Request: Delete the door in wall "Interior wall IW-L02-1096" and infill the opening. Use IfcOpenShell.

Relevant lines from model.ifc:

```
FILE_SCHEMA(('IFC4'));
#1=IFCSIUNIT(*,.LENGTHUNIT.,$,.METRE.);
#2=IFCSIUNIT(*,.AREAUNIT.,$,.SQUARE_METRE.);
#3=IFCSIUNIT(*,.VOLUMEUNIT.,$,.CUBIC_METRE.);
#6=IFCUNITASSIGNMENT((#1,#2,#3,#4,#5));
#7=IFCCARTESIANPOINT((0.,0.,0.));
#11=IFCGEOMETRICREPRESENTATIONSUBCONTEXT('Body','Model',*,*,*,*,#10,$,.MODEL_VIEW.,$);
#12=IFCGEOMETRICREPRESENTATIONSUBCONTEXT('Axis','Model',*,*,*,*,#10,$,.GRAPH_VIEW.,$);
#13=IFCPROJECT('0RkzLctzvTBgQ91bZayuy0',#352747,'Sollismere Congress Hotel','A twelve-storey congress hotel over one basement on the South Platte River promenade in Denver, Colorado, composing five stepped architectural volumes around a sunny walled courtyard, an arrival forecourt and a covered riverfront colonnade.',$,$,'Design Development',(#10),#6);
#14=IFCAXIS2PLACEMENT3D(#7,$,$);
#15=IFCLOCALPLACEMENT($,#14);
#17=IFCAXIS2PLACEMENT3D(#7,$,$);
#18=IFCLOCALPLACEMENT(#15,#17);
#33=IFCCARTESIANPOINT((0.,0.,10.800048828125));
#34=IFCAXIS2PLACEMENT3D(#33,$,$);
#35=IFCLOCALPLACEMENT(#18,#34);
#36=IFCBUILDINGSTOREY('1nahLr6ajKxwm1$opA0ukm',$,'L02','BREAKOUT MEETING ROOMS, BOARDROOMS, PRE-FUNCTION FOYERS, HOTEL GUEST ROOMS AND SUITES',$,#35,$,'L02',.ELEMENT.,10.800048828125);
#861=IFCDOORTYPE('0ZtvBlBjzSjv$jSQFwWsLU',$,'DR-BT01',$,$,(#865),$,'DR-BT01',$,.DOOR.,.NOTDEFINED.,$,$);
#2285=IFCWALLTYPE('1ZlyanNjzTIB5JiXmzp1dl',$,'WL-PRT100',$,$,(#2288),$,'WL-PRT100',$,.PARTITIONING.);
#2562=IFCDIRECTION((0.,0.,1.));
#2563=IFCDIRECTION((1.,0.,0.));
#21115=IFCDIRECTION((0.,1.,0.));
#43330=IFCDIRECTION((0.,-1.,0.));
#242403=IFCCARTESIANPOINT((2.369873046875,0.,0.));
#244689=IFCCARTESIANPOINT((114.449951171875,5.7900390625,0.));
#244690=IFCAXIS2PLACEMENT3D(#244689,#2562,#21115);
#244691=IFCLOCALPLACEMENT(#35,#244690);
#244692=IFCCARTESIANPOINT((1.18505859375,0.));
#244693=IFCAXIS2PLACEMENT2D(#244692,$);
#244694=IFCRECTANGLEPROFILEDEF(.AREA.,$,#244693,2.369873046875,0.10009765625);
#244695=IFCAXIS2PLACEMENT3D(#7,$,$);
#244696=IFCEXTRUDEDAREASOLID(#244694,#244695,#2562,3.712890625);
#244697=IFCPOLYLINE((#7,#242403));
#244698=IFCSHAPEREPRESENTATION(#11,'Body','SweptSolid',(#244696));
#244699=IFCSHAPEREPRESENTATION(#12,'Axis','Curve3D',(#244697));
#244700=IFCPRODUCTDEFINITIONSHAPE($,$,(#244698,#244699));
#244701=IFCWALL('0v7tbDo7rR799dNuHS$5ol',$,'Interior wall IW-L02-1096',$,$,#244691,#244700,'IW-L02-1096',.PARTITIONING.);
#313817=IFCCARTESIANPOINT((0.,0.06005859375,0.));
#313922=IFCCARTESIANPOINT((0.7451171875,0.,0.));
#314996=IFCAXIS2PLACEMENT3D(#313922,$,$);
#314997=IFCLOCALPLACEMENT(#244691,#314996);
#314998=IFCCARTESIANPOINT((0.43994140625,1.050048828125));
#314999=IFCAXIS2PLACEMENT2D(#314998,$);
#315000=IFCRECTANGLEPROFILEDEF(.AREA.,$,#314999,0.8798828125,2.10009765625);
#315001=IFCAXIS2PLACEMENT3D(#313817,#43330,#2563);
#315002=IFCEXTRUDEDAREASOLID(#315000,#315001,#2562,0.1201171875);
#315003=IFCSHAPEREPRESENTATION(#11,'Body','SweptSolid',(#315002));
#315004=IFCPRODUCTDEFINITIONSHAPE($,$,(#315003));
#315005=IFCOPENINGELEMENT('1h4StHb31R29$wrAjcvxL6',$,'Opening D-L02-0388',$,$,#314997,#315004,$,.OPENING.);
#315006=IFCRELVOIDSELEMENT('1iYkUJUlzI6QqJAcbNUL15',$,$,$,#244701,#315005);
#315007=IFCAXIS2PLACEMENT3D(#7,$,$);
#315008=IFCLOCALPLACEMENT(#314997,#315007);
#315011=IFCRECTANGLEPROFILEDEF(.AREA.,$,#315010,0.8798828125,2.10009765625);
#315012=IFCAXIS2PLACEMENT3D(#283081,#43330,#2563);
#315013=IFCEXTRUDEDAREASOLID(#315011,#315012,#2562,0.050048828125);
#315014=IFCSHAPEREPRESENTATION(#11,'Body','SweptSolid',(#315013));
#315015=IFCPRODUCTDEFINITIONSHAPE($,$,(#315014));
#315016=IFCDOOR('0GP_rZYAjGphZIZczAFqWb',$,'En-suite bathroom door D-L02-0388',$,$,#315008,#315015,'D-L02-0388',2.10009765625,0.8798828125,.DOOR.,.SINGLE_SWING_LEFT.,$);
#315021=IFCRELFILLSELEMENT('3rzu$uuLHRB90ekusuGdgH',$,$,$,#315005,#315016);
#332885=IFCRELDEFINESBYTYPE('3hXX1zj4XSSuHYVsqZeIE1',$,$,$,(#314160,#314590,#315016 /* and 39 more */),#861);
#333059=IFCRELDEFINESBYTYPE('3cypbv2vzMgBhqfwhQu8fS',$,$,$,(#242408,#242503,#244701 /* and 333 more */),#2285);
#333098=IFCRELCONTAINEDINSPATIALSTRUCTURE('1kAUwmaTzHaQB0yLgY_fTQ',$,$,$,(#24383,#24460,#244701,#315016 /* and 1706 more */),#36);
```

```python
import ifcopenshell
import ifcopenshell.api.feature
import ifcopenshell.api.root
import ifcopenshell.geom
import ifcopenshell.util.shape

model = ifcopenshell.open("model.ifc")
settings = ifcopenshell.geom.settings()


def volume(element):
    """Net volume in cubic metres, openings subtracted."""
    shape = ifcopenshell.geom.create_shape(settings, element)
    return ifcopenshell.util.shape.get_volume(shape.geometry)


door = model.by_guid("0GP_rZYAjGphZIZczAFqWb")
opening = door.FillsVoids[0].RelatingOpeningElement
wall = opening.VoidsElements[0].RelatingBuildingElement
before = volume(wall)

ifcopenshell.api.root.remove_product(model, product=door)
ifcopenshell.api.feature.remove_feature(model, feature=opening)

after = volume(wall)

print(f"wall volume {before:.3f} -> {after:.3f} m3")

model.write("model-out.ifc")
```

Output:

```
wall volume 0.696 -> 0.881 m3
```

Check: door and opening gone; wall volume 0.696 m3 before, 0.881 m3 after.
